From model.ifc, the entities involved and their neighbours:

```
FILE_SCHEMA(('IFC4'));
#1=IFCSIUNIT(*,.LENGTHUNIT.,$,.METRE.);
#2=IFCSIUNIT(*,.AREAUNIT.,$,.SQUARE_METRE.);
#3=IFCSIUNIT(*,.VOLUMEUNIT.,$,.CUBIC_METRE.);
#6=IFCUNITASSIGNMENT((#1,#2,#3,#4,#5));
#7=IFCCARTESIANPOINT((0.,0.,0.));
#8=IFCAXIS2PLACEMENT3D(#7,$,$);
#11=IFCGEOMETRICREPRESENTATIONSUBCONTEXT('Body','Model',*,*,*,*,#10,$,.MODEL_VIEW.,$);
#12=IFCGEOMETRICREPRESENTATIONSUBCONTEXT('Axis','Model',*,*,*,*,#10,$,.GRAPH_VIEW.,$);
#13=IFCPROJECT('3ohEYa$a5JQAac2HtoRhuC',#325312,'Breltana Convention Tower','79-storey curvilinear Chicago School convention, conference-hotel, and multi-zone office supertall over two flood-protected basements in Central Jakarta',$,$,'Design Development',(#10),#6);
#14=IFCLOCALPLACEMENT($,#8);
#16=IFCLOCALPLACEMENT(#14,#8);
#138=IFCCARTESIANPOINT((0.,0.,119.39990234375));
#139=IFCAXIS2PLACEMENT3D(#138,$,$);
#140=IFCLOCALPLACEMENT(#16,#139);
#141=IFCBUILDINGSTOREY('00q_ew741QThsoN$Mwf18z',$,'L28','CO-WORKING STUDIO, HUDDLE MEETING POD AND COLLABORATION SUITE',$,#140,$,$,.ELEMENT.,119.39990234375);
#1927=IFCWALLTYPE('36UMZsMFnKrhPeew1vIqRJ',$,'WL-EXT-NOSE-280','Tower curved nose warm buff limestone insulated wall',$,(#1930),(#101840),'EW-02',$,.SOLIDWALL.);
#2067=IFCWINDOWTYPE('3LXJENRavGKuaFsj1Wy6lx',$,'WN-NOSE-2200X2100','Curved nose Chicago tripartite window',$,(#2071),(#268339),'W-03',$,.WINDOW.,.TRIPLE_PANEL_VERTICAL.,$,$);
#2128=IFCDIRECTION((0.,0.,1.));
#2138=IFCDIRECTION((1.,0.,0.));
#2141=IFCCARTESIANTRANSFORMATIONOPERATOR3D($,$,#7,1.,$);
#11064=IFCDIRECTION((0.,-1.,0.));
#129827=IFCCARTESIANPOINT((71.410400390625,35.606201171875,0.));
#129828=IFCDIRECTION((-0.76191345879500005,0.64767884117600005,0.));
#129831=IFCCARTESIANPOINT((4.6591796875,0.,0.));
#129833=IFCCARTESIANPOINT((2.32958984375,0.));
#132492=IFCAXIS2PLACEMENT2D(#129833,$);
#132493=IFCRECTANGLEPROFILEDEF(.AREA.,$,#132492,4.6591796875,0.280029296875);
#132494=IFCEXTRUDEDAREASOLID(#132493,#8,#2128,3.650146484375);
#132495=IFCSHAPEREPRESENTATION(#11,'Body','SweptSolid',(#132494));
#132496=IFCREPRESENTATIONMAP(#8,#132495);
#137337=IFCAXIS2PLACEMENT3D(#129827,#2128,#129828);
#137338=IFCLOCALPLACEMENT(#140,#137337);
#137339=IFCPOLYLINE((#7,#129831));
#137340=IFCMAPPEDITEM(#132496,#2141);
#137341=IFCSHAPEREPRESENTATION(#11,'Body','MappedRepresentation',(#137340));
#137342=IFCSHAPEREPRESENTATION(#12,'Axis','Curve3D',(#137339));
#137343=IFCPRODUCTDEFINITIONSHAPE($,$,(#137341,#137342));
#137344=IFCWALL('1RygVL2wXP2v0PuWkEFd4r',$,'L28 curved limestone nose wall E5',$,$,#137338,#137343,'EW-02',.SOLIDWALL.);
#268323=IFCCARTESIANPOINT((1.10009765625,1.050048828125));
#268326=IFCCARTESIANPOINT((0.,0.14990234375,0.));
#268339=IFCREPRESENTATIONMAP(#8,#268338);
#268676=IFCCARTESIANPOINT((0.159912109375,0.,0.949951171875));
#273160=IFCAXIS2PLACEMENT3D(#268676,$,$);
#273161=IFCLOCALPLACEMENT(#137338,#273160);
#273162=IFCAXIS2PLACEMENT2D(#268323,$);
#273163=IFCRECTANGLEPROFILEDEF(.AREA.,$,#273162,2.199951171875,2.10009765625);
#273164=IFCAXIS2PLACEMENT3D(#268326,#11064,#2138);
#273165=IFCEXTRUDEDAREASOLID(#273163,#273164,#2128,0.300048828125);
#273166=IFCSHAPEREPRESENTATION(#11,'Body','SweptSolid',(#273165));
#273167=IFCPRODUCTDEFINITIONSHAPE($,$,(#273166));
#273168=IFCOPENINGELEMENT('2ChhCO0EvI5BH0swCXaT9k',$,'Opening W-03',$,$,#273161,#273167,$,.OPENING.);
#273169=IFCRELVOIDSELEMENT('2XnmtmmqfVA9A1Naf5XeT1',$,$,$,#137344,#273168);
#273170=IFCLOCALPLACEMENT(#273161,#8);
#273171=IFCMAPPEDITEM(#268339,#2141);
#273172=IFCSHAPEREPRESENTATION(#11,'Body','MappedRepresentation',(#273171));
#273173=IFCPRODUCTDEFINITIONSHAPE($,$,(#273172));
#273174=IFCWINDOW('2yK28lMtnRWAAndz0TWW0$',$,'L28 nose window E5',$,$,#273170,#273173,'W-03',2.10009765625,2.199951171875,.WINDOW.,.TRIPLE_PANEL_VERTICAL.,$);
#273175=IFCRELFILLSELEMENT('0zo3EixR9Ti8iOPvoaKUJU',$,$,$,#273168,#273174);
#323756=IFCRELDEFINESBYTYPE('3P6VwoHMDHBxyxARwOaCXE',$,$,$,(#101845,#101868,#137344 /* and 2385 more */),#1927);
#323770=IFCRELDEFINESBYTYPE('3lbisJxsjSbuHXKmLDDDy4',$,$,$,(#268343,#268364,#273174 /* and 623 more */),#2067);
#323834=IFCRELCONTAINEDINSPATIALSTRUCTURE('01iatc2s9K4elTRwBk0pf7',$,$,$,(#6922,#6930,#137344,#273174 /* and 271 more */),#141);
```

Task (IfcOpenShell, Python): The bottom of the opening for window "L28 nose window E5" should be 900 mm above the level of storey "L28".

```python
import numpy as np
import ifcopenshell
import ifcopenshell.api.geometry
import ifcopenshell.geom
import ifcopenshell.util.element
import ifcopenshell.util.placement
import ifcopenshell.util.shape
import ifcopenshell.util.unit

model = ifcopenshell.open("model.ifc")
unit_scale = ifcopenshell.util.unit.calculate_unit_scale(model)

window = model.by_guid("2yK28lMtnRWAAndz0TWW0$")
opening = window.FillsVoids[0].RelatingOpeningElement
storey = ifcopenshell.util.element.get_container(window, ifc_class="IfcBuildingStorey")
level = ifcopenshell.util.placement.get_local_placement(storey.ObjectPlacement)[2, 3]

# The opening's origin need not be at the sill, so measure its lowest point.
shape = ifcopenshell.geom.create_shape(ifcopenshell.geom.settings(), opening)
bottom = ifcopenshell.util.shape.get_shape_bottom_elevation(shape, shape.geometry) / unit_scale
dz = level + 0.9 - bottom

shift = np.array([0.0, 0.0, dz])
# The window is placed relative to its opening, so it follows when the opening moves.
matrix = ifcopenshell.util.placement.get_local_placement(opening.ObjectPlacement)
matrix[:3, 3] += shift
ifcopenshell.api.geometry.edit_object_placement(
    model, product=opening, matrix=matrix, is_si=False, should_transform_children=True
)

print(f"moved by {dz * unit_scale:+.3f} m")

model.write("model_updated.ifc")
```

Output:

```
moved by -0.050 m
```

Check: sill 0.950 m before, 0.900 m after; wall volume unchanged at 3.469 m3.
